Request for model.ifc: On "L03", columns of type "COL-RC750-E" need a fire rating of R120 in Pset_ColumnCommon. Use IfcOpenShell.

First a look at what the model holds.

```python
import ifcopenshell
import ifcopenshell.util.element

model = ifcopenshell.open("model.ifc")
print(model.schema)
storey = next(s for s in model.by_type("IfcBuildingStorey") if s.Name == "L03")
columns = [e for e in ifcopenshell.util.element.get_decomposition(storey) if e.is_a("IfcColumn")]
seen = {}
for e in columns:
    element_type = ifcopenshell.util.element.get_type(e)
    key = (element_type.Name if element_type != e and element_type else None, ifcopenshell.util.element.get_pset(e, "Pset_ColumnCommon", "FireRating"))
    seen[key] = seen.get(key, 0) + 1
for (name, value), count in sorted(seen.items(), key=str):
    print(count, "x", name, "|", value)
```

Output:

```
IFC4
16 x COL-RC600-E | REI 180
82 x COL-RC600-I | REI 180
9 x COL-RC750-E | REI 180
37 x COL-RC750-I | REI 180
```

```python
import ifcopenshell
import ifcopenshell.api.pset
import ifcopenshell.util.element

model = ifcopenshell.open("model.ifc")

storey = next(s for s in model.by_type("IfcBuildingStorey") if s.Name == "L03")
columns = [e for e in ifcopenshell.util.element.get_decomposition(storey) if e.is_a("IfcColumn")]

count = 0
for e in columns:
    element_type = ifcopenshell.util.element.get_type(e)
    if element_type in (None, e) or element_type.Name != "COL-RC750-E":
        continue
    # add_pset returns the element's existing set when there is one.
    pset = ifcopenshell.api.pset.add_pset(model, product=e, name="Pset_ColumnCommon")
    ifcopenshell.api.pset.edit_pset(model, pset=pset, properties={"FireRating": "R120"})
    count += 1

print(count, "columns updated")

model.write("model_v2.ifc")
```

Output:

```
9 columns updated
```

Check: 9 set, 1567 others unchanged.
